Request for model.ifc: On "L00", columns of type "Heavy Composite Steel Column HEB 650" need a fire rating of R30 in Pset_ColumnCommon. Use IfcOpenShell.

First a look at what the model holds.

```python
import ifcopenshell
import ifcopenshell.util.element

model = ifcopenshell.open("model.ifc")
print(model.schema)
storey = next(s for s in model.by_type("IfcBuildingStorey") if s.Name == "L00")
columns = [e for e in ifcopenshell.util.element.get_decomposition(storey) if e.is_a("IfcColumn")]
seen = {}
for e in columns:
    element_type = ifcopenshell.util.element.get_type(e)
    key = (element_type.Name if element_type != e and element_type else None, ifcopenshell.util.element.get_pset(e, "Pset_ColumnCommon", "FireRating"))
    seen[key] = seen.get(key, 0) + 1
for (name, value), count in sorted(seen.items(), key=str):
    print(count, "x", name, "|", value)
```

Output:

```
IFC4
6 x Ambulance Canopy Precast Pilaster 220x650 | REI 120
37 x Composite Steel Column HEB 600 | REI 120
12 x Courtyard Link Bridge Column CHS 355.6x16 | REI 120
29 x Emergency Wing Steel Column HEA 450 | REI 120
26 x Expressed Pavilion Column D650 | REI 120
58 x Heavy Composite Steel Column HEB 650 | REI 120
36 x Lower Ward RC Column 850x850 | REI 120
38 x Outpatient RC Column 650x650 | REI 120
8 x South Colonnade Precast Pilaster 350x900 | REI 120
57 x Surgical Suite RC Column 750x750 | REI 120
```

```python
import ifcopenshell
import ifcopenshell.api.pset
import ifcopenshell.util.element

model = ifcopenshell.open("model.ifc")

storey = next(s for s in model.by_type("IfcBuildingStorey") if s.Name == "L00")
columns = [e for e in ifcopenshell.util.element.get_decomposition(storey) if e.is_a("IfcColumn")]

count = 0
for e in columns:
    element_type = ifcopenshell.util.element.get_type(e)
    if element_type in (None, e) or element_type.Name != "Heavy Composite Steel Column HEB 650":
        continue
    # add_pset returns the element's existing set when there is one.
    pset = ifcopenshell.api.pset.add_pset(model, product=e, name="Pset_ColumnCommon")
    ifcopenshell.api.pset.edit_pset(model, pset=pset, properties={"FireRating": "R30"})
    count += 1

print(count, "columns updated")

model.write("model_updated.ifc")
```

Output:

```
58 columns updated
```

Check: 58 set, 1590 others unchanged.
